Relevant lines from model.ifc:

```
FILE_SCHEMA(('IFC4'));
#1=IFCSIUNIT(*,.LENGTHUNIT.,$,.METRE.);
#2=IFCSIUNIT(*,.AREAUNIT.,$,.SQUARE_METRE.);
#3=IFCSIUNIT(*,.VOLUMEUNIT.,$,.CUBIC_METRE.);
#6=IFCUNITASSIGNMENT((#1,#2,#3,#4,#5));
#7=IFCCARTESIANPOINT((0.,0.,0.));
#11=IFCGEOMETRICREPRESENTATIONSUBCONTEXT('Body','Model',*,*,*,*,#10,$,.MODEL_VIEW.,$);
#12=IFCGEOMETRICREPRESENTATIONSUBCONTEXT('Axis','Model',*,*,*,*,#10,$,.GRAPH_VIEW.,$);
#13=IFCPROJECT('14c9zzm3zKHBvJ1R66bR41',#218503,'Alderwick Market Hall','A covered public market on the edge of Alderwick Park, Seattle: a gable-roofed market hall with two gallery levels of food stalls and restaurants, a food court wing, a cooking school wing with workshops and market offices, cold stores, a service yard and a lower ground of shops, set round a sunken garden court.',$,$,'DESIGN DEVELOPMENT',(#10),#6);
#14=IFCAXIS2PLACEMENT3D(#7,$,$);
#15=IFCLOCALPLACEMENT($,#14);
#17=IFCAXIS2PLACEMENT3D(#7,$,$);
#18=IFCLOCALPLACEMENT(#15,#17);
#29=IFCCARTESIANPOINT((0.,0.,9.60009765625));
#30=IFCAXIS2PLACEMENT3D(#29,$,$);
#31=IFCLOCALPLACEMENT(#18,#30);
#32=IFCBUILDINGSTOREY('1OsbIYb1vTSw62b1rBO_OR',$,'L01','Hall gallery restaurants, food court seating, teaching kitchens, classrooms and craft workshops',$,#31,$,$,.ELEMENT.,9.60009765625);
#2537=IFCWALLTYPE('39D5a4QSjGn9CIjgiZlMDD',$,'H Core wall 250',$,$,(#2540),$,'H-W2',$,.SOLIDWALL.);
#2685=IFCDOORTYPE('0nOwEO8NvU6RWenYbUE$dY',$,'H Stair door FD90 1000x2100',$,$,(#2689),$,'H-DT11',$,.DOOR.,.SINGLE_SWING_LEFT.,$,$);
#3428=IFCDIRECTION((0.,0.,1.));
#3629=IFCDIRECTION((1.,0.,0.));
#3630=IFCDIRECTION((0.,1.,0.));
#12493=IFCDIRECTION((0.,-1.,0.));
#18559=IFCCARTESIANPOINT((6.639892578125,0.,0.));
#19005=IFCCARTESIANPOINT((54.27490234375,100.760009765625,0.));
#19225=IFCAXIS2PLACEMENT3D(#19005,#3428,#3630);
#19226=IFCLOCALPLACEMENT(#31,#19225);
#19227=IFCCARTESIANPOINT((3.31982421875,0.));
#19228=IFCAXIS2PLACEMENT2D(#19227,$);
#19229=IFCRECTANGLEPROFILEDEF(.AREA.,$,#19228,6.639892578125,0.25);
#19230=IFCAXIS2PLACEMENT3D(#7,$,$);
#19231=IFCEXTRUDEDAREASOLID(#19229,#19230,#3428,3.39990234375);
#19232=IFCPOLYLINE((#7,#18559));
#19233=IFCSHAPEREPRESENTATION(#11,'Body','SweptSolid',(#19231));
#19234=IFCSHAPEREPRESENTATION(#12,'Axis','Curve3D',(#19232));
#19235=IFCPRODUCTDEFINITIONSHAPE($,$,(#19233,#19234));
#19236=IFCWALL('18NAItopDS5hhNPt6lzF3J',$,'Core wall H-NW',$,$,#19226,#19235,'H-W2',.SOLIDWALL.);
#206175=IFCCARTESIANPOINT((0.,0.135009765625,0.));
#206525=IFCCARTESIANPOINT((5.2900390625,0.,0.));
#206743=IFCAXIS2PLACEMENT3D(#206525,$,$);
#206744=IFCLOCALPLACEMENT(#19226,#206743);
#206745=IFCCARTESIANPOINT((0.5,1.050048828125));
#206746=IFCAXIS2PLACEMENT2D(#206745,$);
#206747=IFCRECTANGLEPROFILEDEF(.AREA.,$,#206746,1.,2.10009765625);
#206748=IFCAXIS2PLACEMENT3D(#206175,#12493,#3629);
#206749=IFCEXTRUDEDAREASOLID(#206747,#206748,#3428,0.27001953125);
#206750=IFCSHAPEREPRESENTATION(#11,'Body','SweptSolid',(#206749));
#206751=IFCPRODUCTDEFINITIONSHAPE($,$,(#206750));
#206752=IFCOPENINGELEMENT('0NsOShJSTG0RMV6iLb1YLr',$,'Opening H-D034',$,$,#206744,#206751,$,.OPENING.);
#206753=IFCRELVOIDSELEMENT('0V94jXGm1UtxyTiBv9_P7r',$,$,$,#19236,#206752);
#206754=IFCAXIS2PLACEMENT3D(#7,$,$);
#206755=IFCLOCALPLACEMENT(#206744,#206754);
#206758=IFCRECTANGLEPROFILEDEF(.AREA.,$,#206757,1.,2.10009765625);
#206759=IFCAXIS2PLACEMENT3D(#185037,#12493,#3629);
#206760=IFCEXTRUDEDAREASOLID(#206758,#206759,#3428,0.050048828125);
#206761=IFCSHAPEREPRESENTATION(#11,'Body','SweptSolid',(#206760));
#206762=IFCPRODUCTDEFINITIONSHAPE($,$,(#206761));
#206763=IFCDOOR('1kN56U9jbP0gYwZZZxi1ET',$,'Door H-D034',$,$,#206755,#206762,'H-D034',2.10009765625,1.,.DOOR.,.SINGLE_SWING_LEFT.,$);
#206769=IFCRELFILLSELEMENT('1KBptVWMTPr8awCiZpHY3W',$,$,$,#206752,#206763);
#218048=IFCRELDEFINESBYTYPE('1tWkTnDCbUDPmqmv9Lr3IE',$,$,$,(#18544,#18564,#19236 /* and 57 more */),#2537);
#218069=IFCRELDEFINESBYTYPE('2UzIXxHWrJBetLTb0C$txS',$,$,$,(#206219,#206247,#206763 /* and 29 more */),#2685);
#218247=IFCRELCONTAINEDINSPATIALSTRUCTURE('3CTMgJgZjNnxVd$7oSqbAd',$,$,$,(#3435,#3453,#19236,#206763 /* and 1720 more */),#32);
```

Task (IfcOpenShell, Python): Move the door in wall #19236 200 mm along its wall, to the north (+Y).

```python
import ifcopenshell
import ifcopenshell.api.geometry
import ifcopenshell.util.placement
import ifcopenshell.util.unit

model = ifcopenshell.open("model.ifc")
unit_scale = ifcopenshell.util.unit.calculate_unit_scale(model)

door = model.by_guid("1kN56U9jbP0gYwZZZxi1ET")
opening = door.FillsVoids[0].RelatingOpeningElement
wall = opening.VoidsElements[0].RelatingBuildingElement

wall_matrix = ifcopenshell.util.placement.get_local_placement(wall.ObjectPlacement)
shift = wall_matrix[:3, 0] * 0.2 / unit_scale
before = ifcopenshell.util.placement.get_local_placement(door.ObjectPlacement)[:3, 3].copy()

# The door is placed relative to its opening, so it follows when the opening moves.
matrix = ifcopenshell.util.placement.get_local_placement(opening.ObjectPlacement)
matrix[:3, 3] += shift
ifcopenshell.api.geometry.edit_object_placement(
    model, product=opening, matrix=matrix, is_si=False, should_transform_children=True
)

after = ifcopenshell.util.placement.get_local_placement(door.ObjectPlacement)[:3, 3]
print("door moved by", (after - before).round(3) + 0.0)

model.write("model_edited.ifc")
```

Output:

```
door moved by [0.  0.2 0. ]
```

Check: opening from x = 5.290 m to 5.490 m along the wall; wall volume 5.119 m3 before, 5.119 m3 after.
